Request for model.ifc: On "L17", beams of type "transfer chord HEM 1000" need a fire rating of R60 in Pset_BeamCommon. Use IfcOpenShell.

First a look at what the model holds.

```python
import ifcopenshell
import ifcopenshell.util.element

model = ifcopenshell.open("model.ifc")
print(model.schema)
storey = next(s for s in model.by_type("IfcBuildingStorey") if s.Name == "L17")
beams = [e for e in ifcopenshell.util.element.get_decomposition(storey) if e.is_a("IfcBeam")]
seen = {}
for e in beams:
    element_type = ifcopenshell.util.element.get_type(e)
    key = (element_type.Name if element_type != e and element_type else None, ifcopenshell.util.element.get_pset(e, "Pset_BeamCommon", "FireRating"))
    seen[key] = seen.get(key, 0) + 1
for (name, value), count in sorted(seen.items(), key=str):
    print(count, "x", name, "|", value)
```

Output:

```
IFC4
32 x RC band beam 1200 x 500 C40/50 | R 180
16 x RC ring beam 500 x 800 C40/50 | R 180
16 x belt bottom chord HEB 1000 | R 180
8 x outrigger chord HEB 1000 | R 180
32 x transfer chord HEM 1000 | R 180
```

```python
import ifcopenshell
import ifcopenshell.api.pset
import ifcopenshell.util.element

model = ifcopenshell.open("model.ifc")

storey = next(s for s in model.by_type("IfcBuildingStorey") if s.Name == "L17")
beams = [e for e in ifcopenshell.util.element.get_decomposition(storey) if e.is_a("IfcBeam")]

count = 0
for e in beams:
    element_type = ifcopenshell.util.element.get_type(e)
    if element_type in (None, e) or element_type.Name != "transfer chord HEM 1000":
        continue
    found = ifcopenshell.util.element.get_pset(e, "Pset_BeamCommon", should_inherit=False)
    if found:
        pset = model.by_id(found["id"])
        if len(ifcopenshell.util.element.get_elements_by_pset(pset)) > 1:
            pset = ifcopenshell.api.pset.unshare_pset(model, products=[e], pset=pset)[0]
    else:
        pset = ifcopenshell.api.pset.add_pset(model, product=e, name="Pset_BeamCommon")
    ifcopenshell.api.pset.edit_pset(model, pset=pset, properties={"FireRating": "R60"})
    count += 1

print(count, "beams updated")

model.write("model_updated.ifc")
```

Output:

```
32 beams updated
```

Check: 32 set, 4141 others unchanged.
